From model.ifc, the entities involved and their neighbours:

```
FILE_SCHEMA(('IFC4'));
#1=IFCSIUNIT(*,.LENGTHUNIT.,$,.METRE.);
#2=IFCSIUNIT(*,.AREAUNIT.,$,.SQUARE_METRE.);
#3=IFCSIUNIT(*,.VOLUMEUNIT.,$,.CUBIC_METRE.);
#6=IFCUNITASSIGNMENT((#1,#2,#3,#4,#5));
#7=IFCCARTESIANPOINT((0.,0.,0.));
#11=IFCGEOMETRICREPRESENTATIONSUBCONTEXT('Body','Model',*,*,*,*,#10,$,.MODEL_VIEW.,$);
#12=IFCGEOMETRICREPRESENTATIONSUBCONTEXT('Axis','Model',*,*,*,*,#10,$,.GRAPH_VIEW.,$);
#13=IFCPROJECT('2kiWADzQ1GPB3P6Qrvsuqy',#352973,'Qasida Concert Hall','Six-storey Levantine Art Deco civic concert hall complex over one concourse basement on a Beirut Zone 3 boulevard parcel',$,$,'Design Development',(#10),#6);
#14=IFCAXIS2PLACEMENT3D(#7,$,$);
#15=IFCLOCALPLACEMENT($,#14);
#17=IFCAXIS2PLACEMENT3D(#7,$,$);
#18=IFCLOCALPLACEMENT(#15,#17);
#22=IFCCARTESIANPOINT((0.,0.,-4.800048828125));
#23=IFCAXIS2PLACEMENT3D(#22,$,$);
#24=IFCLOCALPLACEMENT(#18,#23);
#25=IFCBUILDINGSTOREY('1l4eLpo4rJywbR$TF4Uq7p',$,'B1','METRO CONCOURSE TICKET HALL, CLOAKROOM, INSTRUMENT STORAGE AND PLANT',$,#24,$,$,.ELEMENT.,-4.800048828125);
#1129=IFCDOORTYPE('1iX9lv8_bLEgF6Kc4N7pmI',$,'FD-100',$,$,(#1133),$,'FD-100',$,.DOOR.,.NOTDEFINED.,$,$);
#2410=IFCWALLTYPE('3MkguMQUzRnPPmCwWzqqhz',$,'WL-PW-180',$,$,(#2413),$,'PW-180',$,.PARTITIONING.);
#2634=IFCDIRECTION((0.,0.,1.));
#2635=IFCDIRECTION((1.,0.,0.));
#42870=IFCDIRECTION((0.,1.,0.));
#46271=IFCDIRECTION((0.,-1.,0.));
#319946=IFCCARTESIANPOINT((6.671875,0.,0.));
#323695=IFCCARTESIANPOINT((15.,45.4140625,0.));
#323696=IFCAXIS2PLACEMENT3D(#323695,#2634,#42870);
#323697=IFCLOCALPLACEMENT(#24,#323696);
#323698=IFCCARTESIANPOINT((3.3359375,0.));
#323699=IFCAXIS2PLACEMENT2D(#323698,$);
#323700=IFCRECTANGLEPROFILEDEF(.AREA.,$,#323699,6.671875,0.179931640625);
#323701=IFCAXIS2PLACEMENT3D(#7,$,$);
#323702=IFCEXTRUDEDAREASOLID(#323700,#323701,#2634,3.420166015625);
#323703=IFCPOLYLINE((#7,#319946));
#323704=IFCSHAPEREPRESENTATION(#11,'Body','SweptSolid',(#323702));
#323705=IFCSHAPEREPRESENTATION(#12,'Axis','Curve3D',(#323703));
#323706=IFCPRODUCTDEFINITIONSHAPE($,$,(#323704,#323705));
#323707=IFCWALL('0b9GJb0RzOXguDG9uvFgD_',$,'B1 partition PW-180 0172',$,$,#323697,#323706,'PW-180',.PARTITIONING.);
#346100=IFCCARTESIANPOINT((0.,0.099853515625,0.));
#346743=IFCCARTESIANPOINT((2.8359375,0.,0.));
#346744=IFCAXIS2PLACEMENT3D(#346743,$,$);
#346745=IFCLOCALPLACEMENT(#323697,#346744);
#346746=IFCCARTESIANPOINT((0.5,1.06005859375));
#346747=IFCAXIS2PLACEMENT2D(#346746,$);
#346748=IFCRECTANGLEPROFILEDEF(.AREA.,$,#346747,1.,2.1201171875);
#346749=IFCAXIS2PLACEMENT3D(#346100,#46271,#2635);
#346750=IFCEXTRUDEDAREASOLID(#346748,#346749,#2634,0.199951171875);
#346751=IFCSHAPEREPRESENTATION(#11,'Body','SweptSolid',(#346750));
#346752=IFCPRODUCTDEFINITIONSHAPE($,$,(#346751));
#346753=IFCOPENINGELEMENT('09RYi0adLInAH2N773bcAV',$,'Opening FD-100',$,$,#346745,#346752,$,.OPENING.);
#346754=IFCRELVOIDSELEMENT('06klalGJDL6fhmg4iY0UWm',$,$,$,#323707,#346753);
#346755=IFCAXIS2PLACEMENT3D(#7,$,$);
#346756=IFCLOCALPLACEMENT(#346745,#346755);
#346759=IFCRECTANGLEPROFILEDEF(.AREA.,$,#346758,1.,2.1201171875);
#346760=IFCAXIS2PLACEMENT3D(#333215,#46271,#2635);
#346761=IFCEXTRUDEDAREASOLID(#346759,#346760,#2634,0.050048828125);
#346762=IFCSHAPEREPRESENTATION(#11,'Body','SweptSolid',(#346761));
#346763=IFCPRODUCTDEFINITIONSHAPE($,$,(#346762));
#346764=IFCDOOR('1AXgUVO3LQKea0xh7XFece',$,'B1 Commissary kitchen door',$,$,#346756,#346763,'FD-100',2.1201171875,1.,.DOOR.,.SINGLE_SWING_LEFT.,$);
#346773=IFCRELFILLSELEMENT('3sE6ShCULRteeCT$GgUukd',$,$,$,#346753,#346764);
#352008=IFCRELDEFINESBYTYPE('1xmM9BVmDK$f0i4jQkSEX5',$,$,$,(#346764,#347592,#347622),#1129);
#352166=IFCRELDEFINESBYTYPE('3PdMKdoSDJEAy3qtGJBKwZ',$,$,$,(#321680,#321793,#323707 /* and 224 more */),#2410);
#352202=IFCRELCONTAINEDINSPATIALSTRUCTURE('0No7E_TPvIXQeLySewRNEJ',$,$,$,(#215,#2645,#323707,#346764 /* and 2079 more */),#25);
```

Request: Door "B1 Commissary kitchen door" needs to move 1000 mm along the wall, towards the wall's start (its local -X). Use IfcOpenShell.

```python
import ifcopenshell
import ifcopenshell.api.geometry
import ifcopenshell.util.placement

model = ifcopenshell.open("model.ifc")

door = model.by_guid("1AXgUVO3LQKea0xh7XFece")
opening = door.FillsVoids[0].RelatingOpeningElement
wall = opening.VoidsElements[0].RelatingBuildingElement

wall_matrix = ifcopenshell.util.placement.get_local_placement(wall.ObjectPlacement)
shift = wall_matrix[:3, 0] * -1.0
before = ifcopenshell.util.placement.get_local_placement(door.ObjectPlacement)[:3, 3].copy()

# The door is placed relative to its opening, so it follows when the opening moves.
matrix = ifcopenshell.util.placement.get_local_placement(opening.ObjectPlacement)
matrix[:3, 3] += shift
ifcopenshell.api.geometry.edit_object_placement(
    model, product=opening, matrix=matrix, is_si=False, should_transform_children=True
)

after = ifcopenshell.util.placement.get_local_placement(door.ObjectPlacement)[:3, 3]
print("door moved by", (after - before).round(3) + 0.0)

model.write("model_rev.ifc")
```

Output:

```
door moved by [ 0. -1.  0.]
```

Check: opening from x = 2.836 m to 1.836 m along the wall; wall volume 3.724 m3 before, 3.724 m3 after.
